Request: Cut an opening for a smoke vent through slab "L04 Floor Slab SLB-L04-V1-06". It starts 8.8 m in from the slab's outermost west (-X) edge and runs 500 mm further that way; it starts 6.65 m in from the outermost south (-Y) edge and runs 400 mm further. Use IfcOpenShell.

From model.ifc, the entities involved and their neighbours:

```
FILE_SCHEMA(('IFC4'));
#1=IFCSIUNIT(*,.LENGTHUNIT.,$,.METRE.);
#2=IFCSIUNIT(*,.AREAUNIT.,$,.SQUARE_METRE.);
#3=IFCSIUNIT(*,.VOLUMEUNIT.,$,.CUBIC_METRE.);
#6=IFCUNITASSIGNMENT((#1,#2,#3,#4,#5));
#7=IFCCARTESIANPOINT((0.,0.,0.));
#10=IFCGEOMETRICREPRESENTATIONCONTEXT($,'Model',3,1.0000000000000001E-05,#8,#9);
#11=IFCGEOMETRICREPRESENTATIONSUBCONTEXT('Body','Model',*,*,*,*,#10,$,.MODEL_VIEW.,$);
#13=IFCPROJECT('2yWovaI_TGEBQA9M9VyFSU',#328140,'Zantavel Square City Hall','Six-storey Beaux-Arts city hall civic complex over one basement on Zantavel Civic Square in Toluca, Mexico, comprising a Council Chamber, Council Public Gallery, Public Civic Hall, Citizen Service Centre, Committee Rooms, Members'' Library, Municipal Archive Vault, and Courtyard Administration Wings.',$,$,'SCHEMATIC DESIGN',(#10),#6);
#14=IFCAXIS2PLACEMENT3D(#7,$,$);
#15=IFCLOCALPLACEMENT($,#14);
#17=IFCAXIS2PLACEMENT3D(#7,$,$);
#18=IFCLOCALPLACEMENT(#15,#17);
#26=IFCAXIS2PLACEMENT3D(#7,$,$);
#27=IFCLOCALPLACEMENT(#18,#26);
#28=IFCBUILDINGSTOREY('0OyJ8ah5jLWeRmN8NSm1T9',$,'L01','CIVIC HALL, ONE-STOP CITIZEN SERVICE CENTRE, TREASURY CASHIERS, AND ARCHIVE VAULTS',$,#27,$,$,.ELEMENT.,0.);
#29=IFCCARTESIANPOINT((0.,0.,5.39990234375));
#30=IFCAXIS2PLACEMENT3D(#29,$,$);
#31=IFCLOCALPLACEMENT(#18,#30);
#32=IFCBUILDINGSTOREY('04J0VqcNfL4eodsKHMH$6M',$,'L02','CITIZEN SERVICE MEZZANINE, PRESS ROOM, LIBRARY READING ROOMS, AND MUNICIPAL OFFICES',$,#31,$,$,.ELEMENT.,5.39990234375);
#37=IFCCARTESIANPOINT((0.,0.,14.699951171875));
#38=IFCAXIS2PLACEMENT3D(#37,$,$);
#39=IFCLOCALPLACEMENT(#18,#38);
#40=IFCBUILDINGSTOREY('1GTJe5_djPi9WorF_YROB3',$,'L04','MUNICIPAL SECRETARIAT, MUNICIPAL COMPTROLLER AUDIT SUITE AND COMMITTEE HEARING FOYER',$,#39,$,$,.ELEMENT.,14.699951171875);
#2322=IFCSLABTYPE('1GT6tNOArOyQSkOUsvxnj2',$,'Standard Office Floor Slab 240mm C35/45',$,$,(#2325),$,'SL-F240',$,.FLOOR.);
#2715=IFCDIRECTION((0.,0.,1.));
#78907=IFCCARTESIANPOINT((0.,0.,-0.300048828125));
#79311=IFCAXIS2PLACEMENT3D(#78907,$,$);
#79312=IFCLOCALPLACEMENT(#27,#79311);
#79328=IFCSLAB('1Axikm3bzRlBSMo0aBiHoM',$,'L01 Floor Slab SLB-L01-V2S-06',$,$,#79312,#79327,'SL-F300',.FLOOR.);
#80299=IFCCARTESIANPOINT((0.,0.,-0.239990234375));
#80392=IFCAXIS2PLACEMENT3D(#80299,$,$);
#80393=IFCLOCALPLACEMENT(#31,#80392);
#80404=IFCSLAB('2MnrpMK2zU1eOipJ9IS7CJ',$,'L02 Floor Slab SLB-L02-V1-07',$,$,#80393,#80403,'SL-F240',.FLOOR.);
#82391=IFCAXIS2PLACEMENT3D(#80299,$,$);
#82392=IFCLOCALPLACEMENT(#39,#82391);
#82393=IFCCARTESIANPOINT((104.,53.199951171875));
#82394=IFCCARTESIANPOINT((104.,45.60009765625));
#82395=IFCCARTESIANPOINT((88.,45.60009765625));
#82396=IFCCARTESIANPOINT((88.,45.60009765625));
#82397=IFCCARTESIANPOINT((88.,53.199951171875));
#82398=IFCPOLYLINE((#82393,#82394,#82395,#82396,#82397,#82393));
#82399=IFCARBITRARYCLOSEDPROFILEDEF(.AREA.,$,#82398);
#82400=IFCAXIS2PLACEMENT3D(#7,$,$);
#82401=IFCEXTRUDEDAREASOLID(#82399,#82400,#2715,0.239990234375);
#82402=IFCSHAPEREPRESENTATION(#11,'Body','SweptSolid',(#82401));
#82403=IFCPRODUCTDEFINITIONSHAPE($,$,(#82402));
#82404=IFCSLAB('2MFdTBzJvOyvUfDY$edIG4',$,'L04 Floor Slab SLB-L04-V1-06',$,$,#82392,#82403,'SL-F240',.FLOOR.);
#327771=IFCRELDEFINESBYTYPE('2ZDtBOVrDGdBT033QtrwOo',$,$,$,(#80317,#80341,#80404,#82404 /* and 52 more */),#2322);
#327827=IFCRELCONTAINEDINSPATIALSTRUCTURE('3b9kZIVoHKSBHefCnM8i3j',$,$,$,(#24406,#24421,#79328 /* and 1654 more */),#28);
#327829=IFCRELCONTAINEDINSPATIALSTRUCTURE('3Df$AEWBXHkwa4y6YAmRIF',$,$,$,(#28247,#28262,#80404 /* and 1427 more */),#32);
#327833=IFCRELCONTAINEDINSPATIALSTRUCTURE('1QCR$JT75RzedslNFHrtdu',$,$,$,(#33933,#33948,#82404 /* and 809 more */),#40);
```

```python
import numpy as np
import ifcopenshell
import ifcopenshell.api.feature
import ifcopenshell.api.geometry
import ifcopenshell.api.root
import ifcopenshell.geom
import ifcopenshell.util.placement
import ifcopenshell.util.representation
import ifcopenshell.util.shape
import ifcopenshell.util.unit

model = ifcopenshell.open("model.ifc")
unit_scale = ifcopenshell.util.unit.calculate_unit_scale(model)
settings = ifcopenshell.geom.settings()


def volume(element):
    """Net volume in cubic metres, openings subtracted."""
    shape = ifcopenshell.geom.create_shape(settings, element)
    return ifcopenshell.util.shape.get_volume(shape.geometry)


slab = model.by_guid("2MFdTBzJvOyvUfDY$edIG4")
before = volume(slab)

# Extent in the slab's own axes, in metres. The edges named are its -X and -Y sides.
slab_shape = ifcopenshell.geom.create_shape(settings, slab)
vertices = ifcopenshell.util.shape.get_vertices(slab_shape.geometry)
x_min, y_min, bottom = vertices.min(axis=0)
top = vertices[:, 2].max()

opening = ifcopenshell.api.root.create_entity(model, ifc_class="IfcOpeningElement", name="Smoke vent opening", predefined_type="OPENING")
context = ifcopenshell.util.representation.get_context(model, "Model", "Body", "MODEL_VIEW")
width, depth = 0.5, 0.4
outline = [(0.0, 0.0), (width, 0.0), (width, depth), (0.0, depth), (0.0, 0.0)]
# Overshoot both faces by 50 mm so the cut is clean.
shape = ifcopenshell.api.geometry.add_slab_representation(
    model, context=context, depth=top - bottom + 0.1, polyline=outline
)
ifcopenshell.api.geometry.assign_representation(model, product=opening, representation=shape)

matrix = ifcopenshell.util.placement.get_local_placement(slab.ObjectPlacement)
matrix[:, 3] = matrix @ np.append(np.array([x_min + 8.8, y_min + 6.65, bottom - 0.05]) / unit_scale, 1.0)
ifcopenshell.api.geometry.edit_object_placement(model, product=opening, matrix=matrix, is_si=False)
ifcopenshell.api.feature.add_feature(model, feature=opening, element=slab)

after = volume(slab)

print(f"slab volume {before:.3f} -> {after:.3f} m3")

model.write("model_v2.ifc")
```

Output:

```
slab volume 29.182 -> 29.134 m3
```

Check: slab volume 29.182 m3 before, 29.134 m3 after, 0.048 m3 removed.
